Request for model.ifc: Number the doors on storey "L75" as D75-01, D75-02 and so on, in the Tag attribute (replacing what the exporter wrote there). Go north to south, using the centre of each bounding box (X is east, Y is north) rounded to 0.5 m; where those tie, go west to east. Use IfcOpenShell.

First a look at what the model holds.

```python
import ifcopenshell
import ifcopenshell.util.element
import ifcopenshell.util.placement

model = ifcopenshell.open("model.ifc")
print(model.schema)
storey = next(s for s in model.by_type("IfcBuildingStorey") if s.Name == "L75")
doors = [e for e in ifcopenshell.util.element.get_decomposition(storey) if e.is_a("IfcDoor")]
for e in sorted(doors, key=lambda e: e.id()):
    origin = ifcopenshell.util.placement.get_local_placement(e.ObjectPlacement)[:3, 3]
    print(e.id(), e.Tag, e.Name, origin.round(2) + 0.0, sep=" | ")
```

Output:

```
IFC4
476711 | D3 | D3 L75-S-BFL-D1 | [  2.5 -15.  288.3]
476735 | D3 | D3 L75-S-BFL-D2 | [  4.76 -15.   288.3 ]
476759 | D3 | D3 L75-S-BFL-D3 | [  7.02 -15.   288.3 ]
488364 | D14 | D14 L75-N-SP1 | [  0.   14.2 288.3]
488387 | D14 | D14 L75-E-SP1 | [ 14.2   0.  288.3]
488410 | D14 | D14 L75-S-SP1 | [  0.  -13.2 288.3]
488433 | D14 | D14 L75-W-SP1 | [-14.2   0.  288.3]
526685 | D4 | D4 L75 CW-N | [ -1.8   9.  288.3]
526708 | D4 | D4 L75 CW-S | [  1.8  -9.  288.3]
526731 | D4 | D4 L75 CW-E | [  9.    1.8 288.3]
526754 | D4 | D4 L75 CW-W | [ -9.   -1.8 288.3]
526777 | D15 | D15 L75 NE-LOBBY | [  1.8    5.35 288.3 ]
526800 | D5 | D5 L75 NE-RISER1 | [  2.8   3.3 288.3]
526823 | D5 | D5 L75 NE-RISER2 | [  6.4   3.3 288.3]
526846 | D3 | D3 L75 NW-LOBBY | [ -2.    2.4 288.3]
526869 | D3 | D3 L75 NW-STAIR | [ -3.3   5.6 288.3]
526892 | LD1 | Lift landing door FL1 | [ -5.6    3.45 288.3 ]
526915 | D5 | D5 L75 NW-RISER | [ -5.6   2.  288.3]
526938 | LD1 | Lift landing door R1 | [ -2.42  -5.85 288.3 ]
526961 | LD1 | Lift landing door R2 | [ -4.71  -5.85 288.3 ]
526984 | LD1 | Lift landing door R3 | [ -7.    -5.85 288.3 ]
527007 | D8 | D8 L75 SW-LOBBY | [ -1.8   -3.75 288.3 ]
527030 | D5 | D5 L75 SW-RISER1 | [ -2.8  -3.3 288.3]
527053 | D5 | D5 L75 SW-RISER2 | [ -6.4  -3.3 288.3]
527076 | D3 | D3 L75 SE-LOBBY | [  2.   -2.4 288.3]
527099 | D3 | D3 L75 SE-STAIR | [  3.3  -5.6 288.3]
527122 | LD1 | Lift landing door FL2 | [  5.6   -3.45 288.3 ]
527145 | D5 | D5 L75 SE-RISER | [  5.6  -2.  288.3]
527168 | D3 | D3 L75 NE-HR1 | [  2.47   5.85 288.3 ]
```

```python
import ifcopenshell
import ifcopenshell.geom
import ifcopenshell.util.element
import ifcopenshell.util.shape

model = ifcopenshell.open("model.ifc")
settings = ifcopenshell.geom.settings()
settings.set("use-world-coords", True)


def centre(element):
    shape = ifcopenshell.geom.create_shape(settings, element)
    return ifcopenshell.util.shape.get_bbox_centroid(shape.geometry)


storey = next(s for s in model.by_type("IfcBuildingStorey") if s.Name == "L75")
doors = [e for e in ifcopenshell.util.element.get_decomposition(storey) if e.is_a("IfcDoor")]

# Insertion points can sit at a corner or the storey origin, so sort by the geometry (in metres).
centres = {e: centre(e) for e in doors}
doors.sort(key=lambda e: (-round(centres[e][1] / 0.5), centres[e][0]))

for i, e in enumerate(doors, start=1):
    number = f"D75-{i:02d}"
    e.Tag = number
    print(e.id(), number)

model.write("model_v2.ifc")
```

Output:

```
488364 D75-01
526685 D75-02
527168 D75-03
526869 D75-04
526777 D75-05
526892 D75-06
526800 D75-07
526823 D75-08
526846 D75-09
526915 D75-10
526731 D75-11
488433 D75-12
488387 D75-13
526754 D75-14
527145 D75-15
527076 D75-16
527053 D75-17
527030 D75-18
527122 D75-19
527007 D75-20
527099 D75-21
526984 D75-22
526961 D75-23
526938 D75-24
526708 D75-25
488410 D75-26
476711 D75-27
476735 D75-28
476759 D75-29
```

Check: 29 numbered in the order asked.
